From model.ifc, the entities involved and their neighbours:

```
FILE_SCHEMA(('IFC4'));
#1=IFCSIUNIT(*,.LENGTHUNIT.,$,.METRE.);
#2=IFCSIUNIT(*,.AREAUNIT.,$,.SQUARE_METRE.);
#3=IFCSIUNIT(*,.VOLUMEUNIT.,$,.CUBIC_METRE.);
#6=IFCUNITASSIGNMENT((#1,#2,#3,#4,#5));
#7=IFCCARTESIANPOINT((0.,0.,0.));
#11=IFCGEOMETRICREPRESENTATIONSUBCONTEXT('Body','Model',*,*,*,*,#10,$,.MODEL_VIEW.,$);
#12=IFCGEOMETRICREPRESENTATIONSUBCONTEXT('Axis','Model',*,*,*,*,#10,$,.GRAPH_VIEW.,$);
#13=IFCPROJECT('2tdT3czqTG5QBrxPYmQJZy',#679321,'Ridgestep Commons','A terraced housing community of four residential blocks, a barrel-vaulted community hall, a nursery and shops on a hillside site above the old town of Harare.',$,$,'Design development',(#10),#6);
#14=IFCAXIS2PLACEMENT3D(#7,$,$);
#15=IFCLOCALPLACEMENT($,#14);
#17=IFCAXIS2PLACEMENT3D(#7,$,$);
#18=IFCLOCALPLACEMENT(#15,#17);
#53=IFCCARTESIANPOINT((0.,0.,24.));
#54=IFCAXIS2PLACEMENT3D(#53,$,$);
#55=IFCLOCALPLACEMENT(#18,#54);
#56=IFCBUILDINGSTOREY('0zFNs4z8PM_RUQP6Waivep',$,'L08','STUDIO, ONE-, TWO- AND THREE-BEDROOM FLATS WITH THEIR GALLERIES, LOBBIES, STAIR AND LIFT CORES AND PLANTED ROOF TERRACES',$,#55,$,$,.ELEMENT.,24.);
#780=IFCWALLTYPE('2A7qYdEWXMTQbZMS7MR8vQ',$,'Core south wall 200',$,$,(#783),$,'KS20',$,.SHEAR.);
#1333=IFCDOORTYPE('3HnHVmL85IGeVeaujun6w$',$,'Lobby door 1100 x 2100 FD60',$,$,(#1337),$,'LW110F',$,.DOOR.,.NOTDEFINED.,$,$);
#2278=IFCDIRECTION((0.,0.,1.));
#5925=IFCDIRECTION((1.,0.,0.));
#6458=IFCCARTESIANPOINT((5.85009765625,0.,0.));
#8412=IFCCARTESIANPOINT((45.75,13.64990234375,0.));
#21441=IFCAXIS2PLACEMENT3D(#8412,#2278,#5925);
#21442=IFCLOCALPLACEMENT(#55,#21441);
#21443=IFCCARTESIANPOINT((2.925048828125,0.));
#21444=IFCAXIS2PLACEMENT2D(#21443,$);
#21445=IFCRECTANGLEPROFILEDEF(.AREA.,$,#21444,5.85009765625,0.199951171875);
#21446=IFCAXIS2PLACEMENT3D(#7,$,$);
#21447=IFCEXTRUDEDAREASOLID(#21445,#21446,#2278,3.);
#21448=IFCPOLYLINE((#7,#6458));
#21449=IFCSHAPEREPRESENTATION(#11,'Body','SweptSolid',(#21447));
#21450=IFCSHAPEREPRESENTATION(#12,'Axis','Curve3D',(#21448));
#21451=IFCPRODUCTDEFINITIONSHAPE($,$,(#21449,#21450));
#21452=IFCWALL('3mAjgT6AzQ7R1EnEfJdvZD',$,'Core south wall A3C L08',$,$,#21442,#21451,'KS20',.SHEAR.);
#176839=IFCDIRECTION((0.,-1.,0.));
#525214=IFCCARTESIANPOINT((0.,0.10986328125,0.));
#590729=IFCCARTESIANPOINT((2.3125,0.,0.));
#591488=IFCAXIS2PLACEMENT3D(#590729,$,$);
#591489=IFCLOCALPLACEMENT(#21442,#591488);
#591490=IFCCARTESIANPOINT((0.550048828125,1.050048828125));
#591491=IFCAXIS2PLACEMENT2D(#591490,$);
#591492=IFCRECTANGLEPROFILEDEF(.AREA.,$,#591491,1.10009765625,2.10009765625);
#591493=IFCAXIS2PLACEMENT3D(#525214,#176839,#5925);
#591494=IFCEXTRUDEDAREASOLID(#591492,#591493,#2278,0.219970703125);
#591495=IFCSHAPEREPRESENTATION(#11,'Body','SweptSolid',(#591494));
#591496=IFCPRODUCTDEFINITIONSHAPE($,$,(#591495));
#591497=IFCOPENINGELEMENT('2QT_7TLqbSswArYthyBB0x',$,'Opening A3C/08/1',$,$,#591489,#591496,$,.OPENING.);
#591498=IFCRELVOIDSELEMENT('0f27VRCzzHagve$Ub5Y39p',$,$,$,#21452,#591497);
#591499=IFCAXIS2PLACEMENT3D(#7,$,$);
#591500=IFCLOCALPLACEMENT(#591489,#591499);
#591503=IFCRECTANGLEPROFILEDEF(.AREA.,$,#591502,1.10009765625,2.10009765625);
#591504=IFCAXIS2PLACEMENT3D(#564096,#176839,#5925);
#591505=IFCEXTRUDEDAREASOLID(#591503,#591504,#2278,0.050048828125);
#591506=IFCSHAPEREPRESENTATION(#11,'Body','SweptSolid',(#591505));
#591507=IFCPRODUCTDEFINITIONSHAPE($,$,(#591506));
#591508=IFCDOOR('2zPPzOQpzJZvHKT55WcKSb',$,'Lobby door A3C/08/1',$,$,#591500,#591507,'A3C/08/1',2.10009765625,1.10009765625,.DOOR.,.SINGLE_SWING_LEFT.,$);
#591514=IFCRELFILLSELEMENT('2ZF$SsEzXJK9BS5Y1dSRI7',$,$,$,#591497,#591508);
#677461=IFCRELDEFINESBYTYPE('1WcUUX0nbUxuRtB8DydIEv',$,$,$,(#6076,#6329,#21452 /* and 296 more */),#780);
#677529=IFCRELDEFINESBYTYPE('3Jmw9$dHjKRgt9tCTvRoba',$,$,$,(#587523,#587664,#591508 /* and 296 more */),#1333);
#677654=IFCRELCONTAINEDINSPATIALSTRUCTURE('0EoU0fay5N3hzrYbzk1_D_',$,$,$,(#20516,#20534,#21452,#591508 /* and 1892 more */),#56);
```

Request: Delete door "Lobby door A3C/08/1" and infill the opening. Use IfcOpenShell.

```python
import ifcopenshell
import ifcopenshell.api.feature
import ifcopenshell.api.root
import ifcopenshell.geom
import ifcopenshell.util.shape

model = ifcopenshell.open("model.ifc")
settings = ifcopenshell.geom.settings()


def volume(element):
    """Net volume in cubic metres, openings subtracted."""
    shape = ifcopenshell.geom.create_shape(settings, element)
    return ifcopenshell.util.shape.get_volume(shape.geometry)


door = model.by_guid("2zPPzOQpzJZvHKT55WcKSb")
opening = door.FillsVoids[0].RelatingOpeningElement
wall = opening.VoidsElements[0].RelatingBuildingElement
before = volume(wall)

ifcopenshell.api.root.remove_product(model, product=door)
ifcopenshell.api.feature.remove_feature(model, feature=opening)

after = volume(wall)

print(f"wall volume {before:.3f} -> {after:.3f} m3")

model.write("model_updated.ifc")
```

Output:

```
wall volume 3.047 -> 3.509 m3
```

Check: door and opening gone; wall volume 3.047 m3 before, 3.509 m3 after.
